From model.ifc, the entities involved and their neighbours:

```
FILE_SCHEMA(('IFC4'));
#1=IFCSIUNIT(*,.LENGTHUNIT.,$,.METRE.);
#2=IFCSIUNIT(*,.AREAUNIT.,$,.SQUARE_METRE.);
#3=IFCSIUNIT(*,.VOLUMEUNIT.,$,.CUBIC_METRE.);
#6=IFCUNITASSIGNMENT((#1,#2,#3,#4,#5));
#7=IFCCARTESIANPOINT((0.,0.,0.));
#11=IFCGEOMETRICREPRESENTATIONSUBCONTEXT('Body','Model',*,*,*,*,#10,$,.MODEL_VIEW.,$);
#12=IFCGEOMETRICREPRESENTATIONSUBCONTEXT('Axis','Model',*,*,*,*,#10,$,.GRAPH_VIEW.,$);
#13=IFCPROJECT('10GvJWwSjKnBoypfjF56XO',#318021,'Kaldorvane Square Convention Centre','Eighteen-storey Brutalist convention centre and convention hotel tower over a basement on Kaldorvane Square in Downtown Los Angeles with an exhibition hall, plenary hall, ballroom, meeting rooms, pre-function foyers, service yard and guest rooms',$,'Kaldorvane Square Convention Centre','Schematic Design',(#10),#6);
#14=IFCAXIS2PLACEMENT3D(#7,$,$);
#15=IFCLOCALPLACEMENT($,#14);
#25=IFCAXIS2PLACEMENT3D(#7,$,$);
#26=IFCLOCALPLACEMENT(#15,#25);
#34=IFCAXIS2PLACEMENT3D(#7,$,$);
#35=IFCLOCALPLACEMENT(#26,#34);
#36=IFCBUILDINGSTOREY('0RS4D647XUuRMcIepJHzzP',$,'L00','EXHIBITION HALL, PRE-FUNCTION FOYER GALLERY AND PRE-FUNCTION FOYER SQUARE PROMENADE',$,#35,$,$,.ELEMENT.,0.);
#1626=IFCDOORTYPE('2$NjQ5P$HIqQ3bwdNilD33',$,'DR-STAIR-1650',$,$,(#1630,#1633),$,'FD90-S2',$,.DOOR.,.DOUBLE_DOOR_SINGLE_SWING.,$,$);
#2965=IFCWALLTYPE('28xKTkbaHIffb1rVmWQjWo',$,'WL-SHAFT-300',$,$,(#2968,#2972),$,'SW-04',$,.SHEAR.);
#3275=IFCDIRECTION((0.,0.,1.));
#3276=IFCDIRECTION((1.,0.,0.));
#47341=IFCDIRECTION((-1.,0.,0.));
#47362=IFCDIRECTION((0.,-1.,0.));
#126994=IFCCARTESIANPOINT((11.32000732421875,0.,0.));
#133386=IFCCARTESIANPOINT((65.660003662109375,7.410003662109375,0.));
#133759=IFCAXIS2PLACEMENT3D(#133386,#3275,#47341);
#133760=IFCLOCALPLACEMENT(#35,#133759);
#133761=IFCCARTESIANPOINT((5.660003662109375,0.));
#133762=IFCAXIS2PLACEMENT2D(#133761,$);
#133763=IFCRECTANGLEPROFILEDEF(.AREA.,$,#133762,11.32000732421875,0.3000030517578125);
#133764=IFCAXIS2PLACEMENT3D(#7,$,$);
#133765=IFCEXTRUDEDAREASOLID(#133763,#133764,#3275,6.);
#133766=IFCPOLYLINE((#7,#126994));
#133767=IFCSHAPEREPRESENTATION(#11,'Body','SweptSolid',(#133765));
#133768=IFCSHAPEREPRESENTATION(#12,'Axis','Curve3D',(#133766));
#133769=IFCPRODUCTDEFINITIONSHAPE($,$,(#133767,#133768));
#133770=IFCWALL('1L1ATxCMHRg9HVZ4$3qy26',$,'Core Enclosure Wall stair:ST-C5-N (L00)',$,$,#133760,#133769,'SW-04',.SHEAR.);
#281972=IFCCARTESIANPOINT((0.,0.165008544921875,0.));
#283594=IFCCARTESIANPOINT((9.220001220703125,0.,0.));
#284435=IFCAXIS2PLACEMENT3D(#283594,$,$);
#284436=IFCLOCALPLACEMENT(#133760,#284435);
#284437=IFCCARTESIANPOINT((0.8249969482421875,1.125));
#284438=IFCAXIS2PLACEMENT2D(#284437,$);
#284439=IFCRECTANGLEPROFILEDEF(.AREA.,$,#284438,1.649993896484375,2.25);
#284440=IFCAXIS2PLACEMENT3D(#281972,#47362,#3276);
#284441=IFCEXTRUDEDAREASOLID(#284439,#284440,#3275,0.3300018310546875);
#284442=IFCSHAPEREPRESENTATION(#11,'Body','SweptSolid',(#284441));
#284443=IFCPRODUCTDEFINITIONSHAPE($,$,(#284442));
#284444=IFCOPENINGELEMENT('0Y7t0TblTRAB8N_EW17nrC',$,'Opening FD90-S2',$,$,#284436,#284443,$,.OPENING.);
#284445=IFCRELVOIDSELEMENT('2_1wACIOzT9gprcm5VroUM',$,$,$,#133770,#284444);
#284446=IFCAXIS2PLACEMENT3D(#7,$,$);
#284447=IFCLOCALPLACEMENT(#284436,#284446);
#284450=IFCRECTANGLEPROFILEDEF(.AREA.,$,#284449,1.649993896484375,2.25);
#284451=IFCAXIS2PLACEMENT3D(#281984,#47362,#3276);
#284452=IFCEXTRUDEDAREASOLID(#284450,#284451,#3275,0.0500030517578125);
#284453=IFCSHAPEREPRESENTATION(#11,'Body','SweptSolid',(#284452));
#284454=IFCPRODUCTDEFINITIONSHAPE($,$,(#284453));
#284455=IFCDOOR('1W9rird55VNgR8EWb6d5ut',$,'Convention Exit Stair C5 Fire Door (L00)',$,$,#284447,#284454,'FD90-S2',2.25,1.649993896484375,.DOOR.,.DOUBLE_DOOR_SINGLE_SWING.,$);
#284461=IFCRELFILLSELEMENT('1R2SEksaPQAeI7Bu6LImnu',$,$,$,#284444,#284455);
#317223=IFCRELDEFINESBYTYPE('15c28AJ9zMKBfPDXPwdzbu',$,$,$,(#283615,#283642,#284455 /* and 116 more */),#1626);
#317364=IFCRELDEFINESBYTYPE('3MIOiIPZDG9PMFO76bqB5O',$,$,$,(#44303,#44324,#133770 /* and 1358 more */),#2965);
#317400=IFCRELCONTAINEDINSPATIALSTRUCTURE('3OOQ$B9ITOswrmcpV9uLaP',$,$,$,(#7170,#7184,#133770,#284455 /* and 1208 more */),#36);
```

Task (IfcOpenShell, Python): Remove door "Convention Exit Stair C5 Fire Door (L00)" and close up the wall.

```python
import ifcopenshell
import ifcopenshell.api.feature
import ifcopenshell.api.root
import ifcopenshell.geom
import ifcopenshell.util.shape

model = ifcopenshell.open("model.ifc")
settings = ifcopenshell.geom.settings()


def volume(element):
    """Net volume in cubic metres, openings subtracted."""
    shape = ifcopenshell.geom.create_shape(settings, element)
    return ifcopenshell.util.shape.get_volume(shape.geometry)


door = model.by_guid("1W9rird55VNgR8EWb6d5ut")
opening = door.FillsVoids[0].RelatingOpeningElement
wall = opening.VoidsElements[0].RelatingBuildingElement
before = volume(wall)

ifcopenshell.api.root.remove_product(model, product=door)
ifcopenshell.api.feature.remove_feature(model, feature=opening)

after = volume(wall)

print(f"wall volume {before:.3f} -> {after:.3f} m3")

model.write("model_v2.ifc")
```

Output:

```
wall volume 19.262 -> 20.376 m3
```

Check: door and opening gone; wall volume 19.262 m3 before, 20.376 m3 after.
